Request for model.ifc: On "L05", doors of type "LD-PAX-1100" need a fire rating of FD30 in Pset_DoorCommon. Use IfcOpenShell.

First a look at what the model holds.

```python
import ifcopenshell
import ifcopenshell.util.element

model = ifcopenshell.open("model.ifc")
print(model.schema)
storey = next(s for s in model.by_type("IfcBuildingStorey") if s.Name == "L05")
doors = [e for e in ifcopenshell.util.element.get_decomposition(storey) if e.is_a("IfcDoor")]
seen = {}
for e in doors:
    element_type = ifcopenshell.util.element.get_type(e)
    key = (element_type.Name if element_type != e and element_type else None, ifcopenshell.util.element.get_pset(e, "Pset_DoorCommon", "FireRating"))
    seen[key] = seen.get(key, 0) + 1
for (name, value), count in sorted(seen.items(), key=str):
    print(count, "x", name, "|", value)
```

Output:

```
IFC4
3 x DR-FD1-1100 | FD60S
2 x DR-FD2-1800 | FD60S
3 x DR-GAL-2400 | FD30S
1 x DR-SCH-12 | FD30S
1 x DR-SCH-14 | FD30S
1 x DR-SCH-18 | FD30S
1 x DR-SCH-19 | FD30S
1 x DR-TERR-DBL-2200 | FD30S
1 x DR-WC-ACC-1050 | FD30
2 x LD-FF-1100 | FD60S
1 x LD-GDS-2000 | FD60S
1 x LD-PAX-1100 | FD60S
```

```python
import ifcopenshell
import ifcopenshell.api.pset
import ifcopenshell.util.element

model = ifcopenshell.open("model.ifc")

storey = next(s for s in model.by_type("IfcBuildingStorey") if s.Name == "L05")
doors = [e for e in ifcopenshell.util.element.get_decomposition(storey) if e.is_a("IfcDoor")]

count = 0
for e in doors:
    element_type = ifcopenshell.util.element.get_type(e)
    if element_type in (None, e) or element_type.Name != "LD-PAX-1100":
        continue
    # add_pset returns the element's existing set when there is one.
    pset = ifcopenshell.api.pset.add_pset(model, product=e, name="Pset_DoorCommon")
    ifcopenshell.api.pset.edit_pset(model, pset=pset, properties={"FireRating": "FD30"})
    count += 1

print(count, "doors updated")

model.write("model_rev.ifc")
```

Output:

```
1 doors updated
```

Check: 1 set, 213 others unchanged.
